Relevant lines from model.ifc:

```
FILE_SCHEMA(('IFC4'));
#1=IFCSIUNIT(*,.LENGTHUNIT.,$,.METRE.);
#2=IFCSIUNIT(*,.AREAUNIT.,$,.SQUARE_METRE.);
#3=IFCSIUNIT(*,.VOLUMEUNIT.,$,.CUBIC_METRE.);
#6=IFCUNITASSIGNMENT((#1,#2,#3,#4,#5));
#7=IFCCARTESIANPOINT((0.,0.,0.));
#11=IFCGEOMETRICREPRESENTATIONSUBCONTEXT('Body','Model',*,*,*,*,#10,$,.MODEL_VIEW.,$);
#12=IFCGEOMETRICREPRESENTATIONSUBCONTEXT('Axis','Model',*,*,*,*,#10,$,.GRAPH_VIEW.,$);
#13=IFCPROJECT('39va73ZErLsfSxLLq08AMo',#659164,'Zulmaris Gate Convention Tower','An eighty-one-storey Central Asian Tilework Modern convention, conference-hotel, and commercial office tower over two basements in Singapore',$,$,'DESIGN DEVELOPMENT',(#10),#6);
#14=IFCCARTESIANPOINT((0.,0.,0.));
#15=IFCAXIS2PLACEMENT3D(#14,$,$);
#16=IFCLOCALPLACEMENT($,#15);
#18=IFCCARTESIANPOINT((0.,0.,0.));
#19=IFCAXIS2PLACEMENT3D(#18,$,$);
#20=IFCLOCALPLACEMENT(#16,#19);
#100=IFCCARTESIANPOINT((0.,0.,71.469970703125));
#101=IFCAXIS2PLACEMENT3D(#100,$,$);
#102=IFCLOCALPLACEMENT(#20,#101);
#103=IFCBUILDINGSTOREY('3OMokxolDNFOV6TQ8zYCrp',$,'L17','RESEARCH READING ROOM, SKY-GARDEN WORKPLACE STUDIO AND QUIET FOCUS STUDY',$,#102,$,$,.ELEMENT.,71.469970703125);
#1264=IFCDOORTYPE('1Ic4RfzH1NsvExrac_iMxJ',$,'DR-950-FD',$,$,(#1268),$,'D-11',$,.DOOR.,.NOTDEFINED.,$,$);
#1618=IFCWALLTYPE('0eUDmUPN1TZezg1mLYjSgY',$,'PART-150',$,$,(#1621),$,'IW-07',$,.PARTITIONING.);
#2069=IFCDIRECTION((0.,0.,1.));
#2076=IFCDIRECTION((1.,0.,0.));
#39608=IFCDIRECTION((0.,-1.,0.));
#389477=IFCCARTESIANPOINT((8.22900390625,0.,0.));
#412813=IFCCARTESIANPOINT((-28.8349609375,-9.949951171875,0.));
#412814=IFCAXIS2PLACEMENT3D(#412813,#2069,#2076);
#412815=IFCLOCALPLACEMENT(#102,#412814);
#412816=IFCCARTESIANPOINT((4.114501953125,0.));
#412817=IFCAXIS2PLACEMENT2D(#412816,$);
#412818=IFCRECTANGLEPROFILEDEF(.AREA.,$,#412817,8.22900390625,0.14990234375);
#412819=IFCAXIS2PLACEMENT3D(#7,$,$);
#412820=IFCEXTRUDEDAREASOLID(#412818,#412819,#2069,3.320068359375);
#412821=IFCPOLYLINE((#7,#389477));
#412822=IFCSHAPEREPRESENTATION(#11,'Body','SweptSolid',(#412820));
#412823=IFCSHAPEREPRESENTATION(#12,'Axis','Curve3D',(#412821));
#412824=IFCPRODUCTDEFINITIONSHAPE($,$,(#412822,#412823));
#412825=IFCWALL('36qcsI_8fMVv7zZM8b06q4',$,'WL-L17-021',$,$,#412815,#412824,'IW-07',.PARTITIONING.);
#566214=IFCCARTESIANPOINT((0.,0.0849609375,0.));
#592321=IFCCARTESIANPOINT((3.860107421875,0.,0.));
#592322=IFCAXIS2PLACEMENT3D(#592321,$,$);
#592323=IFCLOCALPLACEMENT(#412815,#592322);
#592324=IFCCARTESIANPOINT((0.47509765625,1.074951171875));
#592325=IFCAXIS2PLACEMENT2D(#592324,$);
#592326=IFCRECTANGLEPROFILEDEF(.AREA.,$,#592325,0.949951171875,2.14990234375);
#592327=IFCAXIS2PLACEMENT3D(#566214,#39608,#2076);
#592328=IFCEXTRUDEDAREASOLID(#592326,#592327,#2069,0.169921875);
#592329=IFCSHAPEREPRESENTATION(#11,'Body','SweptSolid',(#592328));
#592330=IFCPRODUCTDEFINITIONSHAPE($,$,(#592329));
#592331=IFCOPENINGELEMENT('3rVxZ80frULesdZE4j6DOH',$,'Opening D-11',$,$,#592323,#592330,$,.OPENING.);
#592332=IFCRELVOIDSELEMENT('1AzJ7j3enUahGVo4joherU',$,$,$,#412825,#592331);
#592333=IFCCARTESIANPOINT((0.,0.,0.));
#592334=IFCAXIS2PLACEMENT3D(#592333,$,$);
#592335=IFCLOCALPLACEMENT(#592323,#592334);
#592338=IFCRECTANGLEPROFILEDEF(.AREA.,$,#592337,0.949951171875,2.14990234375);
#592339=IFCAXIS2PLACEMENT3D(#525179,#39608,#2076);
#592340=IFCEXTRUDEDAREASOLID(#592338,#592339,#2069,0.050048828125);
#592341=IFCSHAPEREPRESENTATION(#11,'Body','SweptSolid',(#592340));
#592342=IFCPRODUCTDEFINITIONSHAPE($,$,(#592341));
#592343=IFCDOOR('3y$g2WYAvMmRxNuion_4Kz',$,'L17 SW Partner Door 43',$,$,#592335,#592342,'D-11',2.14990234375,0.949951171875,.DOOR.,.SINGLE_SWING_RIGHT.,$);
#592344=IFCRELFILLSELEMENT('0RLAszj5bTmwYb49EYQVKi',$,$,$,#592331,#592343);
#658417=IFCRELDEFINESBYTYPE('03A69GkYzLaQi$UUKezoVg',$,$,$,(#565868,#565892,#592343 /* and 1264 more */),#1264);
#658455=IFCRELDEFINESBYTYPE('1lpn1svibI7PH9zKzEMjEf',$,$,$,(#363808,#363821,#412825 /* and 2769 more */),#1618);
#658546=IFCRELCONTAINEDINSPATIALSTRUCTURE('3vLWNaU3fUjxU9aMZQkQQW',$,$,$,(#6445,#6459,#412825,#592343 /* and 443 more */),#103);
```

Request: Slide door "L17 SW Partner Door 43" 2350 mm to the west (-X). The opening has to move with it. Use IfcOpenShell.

```python
import ifcopenshell
import ifcopenshell.api.geometry
import ifcopenshell.util.placement
import ifcopenshell.util.unit

model = ifcopenshell.open("model.ifc")
unit_scale = ifcopenshell.util.unit.calculate_unit_scale(model)

door = model.by_guid("3y$g2WYAvMmRxNuion_4Kz")
opening = door.FillsVoids[0].RelatingOpeningElement
wall = opening.VoidsElements[0].RelatingBuildingElement

wall_matrix = ifcopenshell.util.placement.get_local_placement(wall.ObjectPlacement)
shift = wall_matrix[:3, 0] * -2.35 / unit_scale
before = ifcopenshell.util.placement.get_local_placement(door.ObjectPlacement)[:3, 3].copy()

# The door is placed relative to its opening, so it follows when the opening moves.
matrix = ifcopenshell.util.placement.get_local_placement(opening.ObjectPlacement)
matrix[:3, 3] += shift
ifcopenshell.api.geometry.edit_object_placement(
    model, product=opening, matrix=matrix, is_si=False, should_transform_children=True
)

after = ifcopenshell.util.placement.get_local_placement(door.ObjectPlacement)[:3, 3]
print("door moved by", (after - before).round(3) + 0.0)

model.write("model_updated.ifc")
```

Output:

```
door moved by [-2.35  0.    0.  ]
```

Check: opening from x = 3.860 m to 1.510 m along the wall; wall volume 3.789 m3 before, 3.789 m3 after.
